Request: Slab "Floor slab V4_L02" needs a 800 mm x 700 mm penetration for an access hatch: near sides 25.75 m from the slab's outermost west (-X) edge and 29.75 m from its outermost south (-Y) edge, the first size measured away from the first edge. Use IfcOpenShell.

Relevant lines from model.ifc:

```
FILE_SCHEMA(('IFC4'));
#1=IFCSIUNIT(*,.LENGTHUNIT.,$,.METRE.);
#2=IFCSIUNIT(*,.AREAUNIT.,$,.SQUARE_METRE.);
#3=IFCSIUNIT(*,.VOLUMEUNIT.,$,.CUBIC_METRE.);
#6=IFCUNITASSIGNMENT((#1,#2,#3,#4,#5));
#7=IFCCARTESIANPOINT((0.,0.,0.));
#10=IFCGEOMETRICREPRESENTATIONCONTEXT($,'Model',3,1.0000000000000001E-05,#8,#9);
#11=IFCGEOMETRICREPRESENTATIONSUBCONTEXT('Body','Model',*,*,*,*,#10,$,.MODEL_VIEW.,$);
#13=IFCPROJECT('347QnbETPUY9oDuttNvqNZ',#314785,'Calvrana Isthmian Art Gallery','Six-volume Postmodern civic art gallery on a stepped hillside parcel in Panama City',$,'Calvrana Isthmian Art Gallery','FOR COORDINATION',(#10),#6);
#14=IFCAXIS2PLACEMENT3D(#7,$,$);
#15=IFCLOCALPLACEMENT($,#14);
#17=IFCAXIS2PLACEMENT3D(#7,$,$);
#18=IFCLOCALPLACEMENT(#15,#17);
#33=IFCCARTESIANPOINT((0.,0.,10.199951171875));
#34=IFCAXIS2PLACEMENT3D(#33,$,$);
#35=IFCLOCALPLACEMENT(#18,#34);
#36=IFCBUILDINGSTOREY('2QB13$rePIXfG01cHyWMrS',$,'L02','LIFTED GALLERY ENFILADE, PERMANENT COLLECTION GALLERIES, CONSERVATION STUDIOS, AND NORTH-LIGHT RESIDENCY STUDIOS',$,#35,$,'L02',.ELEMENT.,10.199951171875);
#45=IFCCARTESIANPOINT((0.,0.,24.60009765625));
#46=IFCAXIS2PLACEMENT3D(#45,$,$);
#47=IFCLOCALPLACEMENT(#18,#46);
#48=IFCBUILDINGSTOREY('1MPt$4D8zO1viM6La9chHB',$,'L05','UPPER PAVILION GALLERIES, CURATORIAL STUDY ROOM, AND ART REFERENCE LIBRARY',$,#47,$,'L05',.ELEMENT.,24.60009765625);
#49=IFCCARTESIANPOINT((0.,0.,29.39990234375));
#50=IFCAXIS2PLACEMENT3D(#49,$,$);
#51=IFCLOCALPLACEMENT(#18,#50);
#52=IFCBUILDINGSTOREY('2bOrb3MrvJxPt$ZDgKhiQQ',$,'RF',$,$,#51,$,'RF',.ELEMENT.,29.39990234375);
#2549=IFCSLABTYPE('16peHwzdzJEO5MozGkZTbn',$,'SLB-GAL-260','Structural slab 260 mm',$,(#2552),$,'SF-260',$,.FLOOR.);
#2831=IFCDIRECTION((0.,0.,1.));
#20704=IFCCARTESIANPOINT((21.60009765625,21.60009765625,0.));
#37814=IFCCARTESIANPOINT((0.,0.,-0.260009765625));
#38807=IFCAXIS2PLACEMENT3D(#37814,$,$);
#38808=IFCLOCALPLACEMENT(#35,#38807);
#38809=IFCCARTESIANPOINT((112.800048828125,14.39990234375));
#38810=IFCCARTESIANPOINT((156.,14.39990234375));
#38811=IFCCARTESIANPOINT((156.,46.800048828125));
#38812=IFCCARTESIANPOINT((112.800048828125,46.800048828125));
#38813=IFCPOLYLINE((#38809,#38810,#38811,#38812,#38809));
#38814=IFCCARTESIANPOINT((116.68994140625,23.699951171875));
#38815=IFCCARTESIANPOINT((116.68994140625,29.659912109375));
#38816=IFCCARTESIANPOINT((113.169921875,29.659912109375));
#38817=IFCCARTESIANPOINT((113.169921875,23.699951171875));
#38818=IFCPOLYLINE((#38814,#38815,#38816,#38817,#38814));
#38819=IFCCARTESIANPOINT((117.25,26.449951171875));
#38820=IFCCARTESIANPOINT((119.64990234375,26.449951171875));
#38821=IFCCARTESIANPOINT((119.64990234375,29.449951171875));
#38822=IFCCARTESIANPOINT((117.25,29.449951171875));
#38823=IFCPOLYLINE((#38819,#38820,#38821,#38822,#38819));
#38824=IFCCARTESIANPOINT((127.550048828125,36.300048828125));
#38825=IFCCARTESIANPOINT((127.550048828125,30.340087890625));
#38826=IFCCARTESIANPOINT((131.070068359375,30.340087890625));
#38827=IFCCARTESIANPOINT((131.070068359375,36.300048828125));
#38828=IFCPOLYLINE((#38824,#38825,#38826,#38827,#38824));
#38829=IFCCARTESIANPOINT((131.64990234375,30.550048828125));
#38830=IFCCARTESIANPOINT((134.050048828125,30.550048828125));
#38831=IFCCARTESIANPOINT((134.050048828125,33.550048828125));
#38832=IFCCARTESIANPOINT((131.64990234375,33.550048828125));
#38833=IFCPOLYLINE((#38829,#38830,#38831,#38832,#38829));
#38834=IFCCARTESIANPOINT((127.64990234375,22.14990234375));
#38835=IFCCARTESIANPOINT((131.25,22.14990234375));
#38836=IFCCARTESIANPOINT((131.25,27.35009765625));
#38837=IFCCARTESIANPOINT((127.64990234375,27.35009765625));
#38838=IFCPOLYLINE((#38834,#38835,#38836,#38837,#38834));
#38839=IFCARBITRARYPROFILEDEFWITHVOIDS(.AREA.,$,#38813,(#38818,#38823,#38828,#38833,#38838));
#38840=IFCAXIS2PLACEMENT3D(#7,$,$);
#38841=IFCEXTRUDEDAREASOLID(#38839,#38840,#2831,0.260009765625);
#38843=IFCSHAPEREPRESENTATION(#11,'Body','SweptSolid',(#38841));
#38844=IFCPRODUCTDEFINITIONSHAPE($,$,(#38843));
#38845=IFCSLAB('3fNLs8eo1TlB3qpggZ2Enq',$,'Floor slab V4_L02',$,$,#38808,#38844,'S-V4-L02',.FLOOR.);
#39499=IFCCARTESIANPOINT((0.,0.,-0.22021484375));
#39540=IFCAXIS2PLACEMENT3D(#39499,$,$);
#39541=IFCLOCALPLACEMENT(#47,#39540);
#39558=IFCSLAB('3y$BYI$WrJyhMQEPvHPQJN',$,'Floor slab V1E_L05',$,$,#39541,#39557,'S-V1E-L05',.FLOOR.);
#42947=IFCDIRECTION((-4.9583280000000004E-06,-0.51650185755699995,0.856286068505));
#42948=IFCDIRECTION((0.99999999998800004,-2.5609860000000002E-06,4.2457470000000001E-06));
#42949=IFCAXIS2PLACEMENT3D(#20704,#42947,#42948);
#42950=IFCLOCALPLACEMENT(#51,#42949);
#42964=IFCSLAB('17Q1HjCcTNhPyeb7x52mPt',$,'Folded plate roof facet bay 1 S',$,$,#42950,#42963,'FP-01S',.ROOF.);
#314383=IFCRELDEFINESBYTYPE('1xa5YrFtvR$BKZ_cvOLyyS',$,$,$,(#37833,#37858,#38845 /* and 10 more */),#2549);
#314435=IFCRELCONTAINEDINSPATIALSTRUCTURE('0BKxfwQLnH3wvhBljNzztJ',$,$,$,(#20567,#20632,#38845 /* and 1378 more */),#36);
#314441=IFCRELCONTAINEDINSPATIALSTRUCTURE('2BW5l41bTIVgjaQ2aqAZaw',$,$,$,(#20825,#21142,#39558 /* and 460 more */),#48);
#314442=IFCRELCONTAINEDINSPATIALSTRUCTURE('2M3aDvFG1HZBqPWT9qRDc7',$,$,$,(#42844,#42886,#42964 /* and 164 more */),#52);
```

```python
import numpy as np
import ifcopenshell
import ifcopenshell.api.feature
import ifcopenshell.api.geometry
import ifcopenshell.api.root
import ifcopenshell.geom
import ifcopenshell.util.placement
import ifcopenshell.util.representation
import ifcopenshell.util.shape
import ifcopenshell.util.unit

model = ifcopenshell.open("model.ifc")
unit_scale = ifcopenshell.util.unit.calculate_unit_scale(model)
settings = ifcopenshell.geom.settings()


def volume(element):
    """Net volume in cubic metres, openings subtracted."""
    shape = ifcopenshell.geom.create_shape(settings, element)
    return ifcopenshell.util.shape.get_volume(shape.geometry)


slab = model.by_guid("3fNLs8eo1TlB3qpggZ2Enq")
before = volume(slab)

# Extent in the slab's own axes, in metres. The edges named are its -X and -Y sides.
slab_shape = ifcopenshell.geom.create_shape(settings, slab)
vertices = ifcopenshell.util.shape.get_vertices(slab_shape.geometry)
x_min, y_min, bottom = vertices.min(axis=0)
top = vertices[:, 2].max()

opening = ifcopenshell.api.root.create_entity(model, ifc_class="IfcOpeningElement", name="Access hatch opening", predefined_type="OPENING")
context = ifcopenshell.util.representation.get_context(model, "Model", "Body", "MODEL_VIEW")
width, depth = 0.8, 0.7
outline = [(0.0, 0.0), (width, 0.0), (width, depth), (0.0, depth), (0.0, 0.0)]
# Overshoot both faces by 50 mm so the cut is clean.
shape = ifcopenshell.api.geometry.add_slab_representation(
    model, context=context, depth=top - bottom + 0.1, polyline=outline
)
ifcopenshell.api.geometry.assign_representation(model, product=opening, representation=shape)

matrix = ifcopenshell.util.placement.get_local_placement(slab.ObjectPlacement)
matrix[:, 3] = matrix @ np.append(np.array([x_min + 25.75, y_min + 29.75, bottom - 0.05]) / unit_scale, 1.0)
ifcopenshell.api.geometry.edit_object_placement(model, product=opening, matrix=matrix, is_si=False)
ifcopenshell.api.feature.add_feature(model, feature=opening, element=slab)

after = volume(slab)

print(f"slab volume {before:.3f} -> {after:.3f} m3")

model.write("model_edited.ifc")
```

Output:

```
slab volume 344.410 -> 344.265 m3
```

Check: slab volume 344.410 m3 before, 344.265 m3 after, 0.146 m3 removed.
